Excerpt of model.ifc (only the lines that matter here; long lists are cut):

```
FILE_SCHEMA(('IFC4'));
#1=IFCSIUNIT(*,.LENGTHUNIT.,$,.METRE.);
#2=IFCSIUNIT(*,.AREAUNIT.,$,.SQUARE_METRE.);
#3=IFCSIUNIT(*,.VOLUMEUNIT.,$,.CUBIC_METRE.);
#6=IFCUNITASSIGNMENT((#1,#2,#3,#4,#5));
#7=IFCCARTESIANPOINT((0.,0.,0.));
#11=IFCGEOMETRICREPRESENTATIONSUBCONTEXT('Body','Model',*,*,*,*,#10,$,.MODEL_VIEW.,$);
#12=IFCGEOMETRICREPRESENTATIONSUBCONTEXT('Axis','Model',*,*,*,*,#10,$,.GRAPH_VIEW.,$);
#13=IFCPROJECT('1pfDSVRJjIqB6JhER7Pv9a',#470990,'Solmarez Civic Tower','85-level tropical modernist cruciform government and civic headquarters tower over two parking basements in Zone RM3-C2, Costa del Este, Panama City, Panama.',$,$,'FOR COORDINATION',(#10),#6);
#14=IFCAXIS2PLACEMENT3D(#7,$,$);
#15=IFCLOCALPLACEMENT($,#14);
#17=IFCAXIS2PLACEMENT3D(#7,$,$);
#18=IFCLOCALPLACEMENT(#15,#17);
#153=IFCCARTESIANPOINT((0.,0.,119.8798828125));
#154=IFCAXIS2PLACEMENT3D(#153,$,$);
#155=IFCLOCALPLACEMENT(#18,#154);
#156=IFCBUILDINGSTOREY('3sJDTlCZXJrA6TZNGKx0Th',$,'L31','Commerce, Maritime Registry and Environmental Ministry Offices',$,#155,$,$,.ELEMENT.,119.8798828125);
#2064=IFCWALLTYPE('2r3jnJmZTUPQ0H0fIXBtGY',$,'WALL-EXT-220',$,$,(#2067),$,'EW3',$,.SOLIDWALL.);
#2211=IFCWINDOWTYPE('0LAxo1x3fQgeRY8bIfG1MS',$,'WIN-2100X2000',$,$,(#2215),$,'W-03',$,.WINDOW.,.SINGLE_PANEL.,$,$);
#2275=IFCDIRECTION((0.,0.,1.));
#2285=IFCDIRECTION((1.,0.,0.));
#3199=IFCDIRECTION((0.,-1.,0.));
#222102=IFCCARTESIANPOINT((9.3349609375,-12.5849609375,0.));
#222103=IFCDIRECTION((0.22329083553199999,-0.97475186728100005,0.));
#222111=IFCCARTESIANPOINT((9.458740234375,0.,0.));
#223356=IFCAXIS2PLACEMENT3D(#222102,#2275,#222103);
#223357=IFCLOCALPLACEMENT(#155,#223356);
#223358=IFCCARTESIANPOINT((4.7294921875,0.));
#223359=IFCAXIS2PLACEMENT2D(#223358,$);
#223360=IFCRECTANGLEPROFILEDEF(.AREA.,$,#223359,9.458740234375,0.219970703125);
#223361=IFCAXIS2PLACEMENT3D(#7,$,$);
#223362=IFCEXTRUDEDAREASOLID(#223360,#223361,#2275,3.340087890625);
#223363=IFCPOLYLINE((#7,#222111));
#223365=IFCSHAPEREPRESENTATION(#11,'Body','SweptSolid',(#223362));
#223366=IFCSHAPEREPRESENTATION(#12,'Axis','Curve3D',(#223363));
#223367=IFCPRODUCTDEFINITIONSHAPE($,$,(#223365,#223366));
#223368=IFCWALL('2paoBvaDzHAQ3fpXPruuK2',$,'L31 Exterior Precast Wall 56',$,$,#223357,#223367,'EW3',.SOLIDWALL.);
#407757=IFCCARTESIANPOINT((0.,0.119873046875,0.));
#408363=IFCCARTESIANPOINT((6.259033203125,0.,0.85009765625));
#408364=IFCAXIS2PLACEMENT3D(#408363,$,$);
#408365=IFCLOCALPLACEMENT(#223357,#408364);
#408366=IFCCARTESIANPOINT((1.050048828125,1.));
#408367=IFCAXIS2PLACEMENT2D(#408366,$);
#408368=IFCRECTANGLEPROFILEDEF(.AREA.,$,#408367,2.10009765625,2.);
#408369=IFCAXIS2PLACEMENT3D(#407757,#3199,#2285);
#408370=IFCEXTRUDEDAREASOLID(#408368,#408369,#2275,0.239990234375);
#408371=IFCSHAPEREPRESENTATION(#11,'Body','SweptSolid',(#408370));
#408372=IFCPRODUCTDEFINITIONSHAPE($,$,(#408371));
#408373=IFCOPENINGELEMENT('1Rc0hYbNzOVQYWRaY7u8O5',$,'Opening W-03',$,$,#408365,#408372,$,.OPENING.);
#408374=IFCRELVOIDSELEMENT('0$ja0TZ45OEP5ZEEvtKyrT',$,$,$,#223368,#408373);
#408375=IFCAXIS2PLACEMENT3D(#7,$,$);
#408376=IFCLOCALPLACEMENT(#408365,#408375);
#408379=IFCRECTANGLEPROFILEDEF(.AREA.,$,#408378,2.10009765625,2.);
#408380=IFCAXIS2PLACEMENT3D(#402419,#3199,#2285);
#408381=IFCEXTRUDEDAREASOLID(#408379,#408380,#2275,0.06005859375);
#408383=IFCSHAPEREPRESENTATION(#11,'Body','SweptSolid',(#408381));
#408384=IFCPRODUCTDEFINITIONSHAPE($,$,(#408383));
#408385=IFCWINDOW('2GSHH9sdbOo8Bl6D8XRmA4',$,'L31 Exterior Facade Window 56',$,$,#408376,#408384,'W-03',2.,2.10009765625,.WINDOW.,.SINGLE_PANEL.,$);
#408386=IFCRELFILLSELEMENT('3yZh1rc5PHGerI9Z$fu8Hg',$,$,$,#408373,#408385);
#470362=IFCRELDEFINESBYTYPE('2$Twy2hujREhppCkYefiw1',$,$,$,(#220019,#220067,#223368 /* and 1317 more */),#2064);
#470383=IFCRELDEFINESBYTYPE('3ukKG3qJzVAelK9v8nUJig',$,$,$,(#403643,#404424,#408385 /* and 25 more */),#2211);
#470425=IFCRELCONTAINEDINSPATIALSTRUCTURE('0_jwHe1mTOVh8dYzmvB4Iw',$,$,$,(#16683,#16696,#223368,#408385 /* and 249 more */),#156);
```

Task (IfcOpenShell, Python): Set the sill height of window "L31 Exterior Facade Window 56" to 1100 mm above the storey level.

```python
import numpy as np
import ifcopenshell
import ifcopenshell.api.geometry
import ifcopenshell.geom
import ifcopenshell.util.element
import ifcopenshell.util.placement
import ifcopenshell.util.shape
import ifcopenshell.util.unit

model = ifcopenshell.open("model.ifc")
unit_scale = ifcopenshell.util.unit.calculate_unit_scale(model)

window = model.by_id(408385)
opening = window.FillsVoids[0].RelatingOpeningElement
storey = ifcopenshell.util.element.get_container(window, ifc_class="IfcBuildingStorey")
level = ifcopenshell.util.placement.get_local_placement(storey.ObjectPlacement)[2, 3]

# The opening's origin need not be at the sill, so measure its lowest point.
shape = ifcopenshell.geom.create_shape(ifcopenshell.geom.settings(), opening)
bottom = ifcopenshell.util.shape.get_shape_bottom_elevation(shape, shape.geometry) / unit_scale
dz = level + 1.1 / unit_scale - bottom

shift = np.array([0.0, 0.0, dz])
# The window is placed relative to its opening, so it follows when the opening moves.
matrix = ifcopenshell.util.placement.get_local_placement(opening.ObjectPlacement)
matrix[:3, 3] += shift
ifcopenshell.api.geometry.edit_object_placement(
    model, product=opening, matrix=matrix, is_si=False, should_transform_children=True
)

print(f"moved by {dz * unit_scale:+.3f} m")

model.write("model_v2.ifc")
```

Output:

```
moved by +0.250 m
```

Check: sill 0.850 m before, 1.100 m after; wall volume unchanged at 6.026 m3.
